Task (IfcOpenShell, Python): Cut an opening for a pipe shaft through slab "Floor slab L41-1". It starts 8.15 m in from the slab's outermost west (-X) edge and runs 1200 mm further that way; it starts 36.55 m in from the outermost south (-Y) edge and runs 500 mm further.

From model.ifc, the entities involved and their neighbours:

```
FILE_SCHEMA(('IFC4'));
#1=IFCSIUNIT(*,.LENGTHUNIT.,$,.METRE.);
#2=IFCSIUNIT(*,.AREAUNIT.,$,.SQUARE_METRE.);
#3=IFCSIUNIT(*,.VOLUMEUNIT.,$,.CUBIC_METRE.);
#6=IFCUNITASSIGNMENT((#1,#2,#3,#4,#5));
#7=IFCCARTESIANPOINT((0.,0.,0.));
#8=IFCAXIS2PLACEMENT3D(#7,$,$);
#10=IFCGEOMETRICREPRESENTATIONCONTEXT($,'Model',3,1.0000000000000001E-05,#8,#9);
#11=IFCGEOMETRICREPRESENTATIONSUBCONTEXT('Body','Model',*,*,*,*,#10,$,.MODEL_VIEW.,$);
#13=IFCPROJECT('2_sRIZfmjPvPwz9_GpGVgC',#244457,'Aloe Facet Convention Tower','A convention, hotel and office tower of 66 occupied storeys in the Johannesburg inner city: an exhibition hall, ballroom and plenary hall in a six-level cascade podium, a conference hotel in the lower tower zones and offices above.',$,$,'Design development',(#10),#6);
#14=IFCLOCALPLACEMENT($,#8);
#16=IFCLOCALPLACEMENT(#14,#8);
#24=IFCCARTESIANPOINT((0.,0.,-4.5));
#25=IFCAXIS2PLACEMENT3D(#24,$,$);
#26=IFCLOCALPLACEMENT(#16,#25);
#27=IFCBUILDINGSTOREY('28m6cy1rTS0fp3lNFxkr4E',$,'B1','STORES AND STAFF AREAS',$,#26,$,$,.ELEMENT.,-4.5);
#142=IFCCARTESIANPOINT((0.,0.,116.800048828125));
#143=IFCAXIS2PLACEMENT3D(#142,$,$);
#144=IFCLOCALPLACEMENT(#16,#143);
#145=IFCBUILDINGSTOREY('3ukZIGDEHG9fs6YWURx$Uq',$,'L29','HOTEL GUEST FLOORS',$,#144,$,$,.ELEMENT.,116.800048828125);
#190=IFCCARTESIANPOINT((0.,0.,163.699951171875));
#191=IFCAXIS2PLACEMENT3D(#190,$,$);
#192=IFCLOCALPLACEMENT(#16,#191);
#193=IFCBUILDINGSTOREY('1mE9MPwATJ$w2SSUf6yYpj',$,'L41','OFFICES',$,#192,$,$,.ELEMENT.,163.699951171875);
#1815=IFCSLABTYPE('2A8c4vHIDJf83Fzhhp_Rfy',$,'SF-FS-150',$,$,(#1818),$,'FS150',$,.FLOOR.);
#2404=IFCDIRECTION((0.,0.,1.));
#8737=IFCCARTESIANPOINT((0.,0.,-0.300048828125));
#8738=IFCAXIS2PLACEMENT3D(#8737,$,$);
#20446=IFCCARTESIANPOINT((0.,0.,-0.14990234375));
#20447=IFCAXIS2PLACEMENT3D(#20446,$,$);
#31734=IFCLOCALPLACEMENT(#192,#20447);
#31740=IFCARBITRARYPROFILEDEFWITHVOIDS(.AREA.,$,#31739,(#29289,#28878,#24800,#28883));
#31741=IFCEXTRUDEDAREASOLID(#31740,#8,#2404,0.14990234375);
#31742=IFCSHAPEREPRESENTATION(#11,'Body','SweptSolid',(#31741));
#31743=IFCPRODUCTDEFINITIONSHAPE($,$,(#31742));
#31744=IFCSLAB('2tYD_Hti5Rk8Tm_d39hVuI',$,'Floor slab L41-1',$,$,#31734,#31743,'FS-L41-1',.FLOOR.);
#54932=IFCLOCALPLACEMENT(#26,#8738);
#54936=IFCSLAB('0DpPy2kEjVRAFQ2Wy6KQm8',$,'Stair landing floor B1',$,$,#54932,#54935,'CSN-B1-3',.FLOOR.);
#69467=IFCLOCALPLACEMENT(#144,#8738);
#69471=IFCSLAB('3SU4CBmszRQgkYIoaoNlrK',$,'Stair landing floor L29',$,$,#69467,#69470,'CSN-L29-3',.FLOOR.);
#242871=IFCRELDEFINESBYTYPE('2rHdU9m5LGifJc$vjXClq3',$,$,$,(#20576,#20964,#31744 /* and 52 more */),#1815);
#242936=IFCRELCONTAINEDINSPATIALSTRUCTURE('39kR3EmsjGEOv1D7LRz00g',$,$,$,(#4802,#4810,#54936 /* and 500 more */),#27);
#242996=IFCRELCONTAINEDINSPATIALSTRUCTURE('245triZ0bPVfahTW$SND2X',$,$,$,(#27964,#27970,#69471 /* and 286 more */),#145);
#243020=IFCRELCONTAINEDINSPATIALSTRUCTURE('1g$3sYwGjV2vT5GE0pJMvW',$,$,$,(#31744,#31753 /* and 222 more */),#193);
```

```python
import numpy as np
import ifcopenshell
import ifcopenshell.api.feature
import ifcopenshell.api.geometry
import ifcopenshell.api.root
import ifcopenshell.geom
import ifcopenshell.util.placement
import ifcopenshell.util.representation
import ifcopenshell.util.shape
import ifcopenshell.util.unit

model = ifcopenshell.open("model.ifc")
unit_scale = ifcopenshell.util.unit.calculate_unit_scale(model)
settings = ifcopenshell.geom.settings()


def volume(element):
    """Net volume in cubic metres, openings subtracted."""
    shape = ifcopenshell.geom.create_shape(settings, element)
    return ifcopenshell.util.shape.get_volume(shape.geometry)


slab = model.by_guid("2tYD_Hti5Rk8Tm_d39hVuI")
before = volume(slab)

# Extent in the slab's own axes, in metres. The edges named are its -X and -Y sides.
slab_shape = ifcopenshell.geom.create_shape(settings, slab)
vertices = ifcopenshell.util.shape.get_vertices(slab_shape.geometry)
x_min, y_min, bottom = vertices.min(axis=0)
top = vertices[:, 2].max()

opening = ifcopenshell.api.root.create_entity(model, ifc_class="IfcOpeningElement", name="Pipe shaft opening", predefined_type="OPENING")
context = ifcopenshell.util.representation.get_context(model, "Model", "Body", "MODEL_VIEW")
width, depth = 1.2, 0.5
outline = [(0.0, 0.0), (width, 0.0), (width, depth), (0.0, depth), (0.0, 0.0)]
# Overshoot both faces by 50 mm so the cut is clean.
shape = ifcopenshell.api.geometry.add_slab_representation(
    model, context=context, depth=top - bottom + 0.1, polyline=outline
)
ifcopenshell.api.geometry.assign_representation(model, product=opening, representation=shape)

matrix = ifcopenshell.util.placement.get_local_placement(slab.ObjectPlacement)
matrix[:, 3] = matrix @ np.append(np.array([x_min + 8.15, y_min + 36.55, bottom - 0.05]) / unit_scale, 1.0)
ifcopenshell.api.geometry.edit_object_placement(model, product=opening, matrix=matrix, is_si=False)
ifcopenshell.api.feature.add_feature(model, feature=opening, element=slab)

after = volume(slab)

print(f"slab volume {before:.3f} -> {after:.3f} m3")

model.write("model_updated.ifc")
```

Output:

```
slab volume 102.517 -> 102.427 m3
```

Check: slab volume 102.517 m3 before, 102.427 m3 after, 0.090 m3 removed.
